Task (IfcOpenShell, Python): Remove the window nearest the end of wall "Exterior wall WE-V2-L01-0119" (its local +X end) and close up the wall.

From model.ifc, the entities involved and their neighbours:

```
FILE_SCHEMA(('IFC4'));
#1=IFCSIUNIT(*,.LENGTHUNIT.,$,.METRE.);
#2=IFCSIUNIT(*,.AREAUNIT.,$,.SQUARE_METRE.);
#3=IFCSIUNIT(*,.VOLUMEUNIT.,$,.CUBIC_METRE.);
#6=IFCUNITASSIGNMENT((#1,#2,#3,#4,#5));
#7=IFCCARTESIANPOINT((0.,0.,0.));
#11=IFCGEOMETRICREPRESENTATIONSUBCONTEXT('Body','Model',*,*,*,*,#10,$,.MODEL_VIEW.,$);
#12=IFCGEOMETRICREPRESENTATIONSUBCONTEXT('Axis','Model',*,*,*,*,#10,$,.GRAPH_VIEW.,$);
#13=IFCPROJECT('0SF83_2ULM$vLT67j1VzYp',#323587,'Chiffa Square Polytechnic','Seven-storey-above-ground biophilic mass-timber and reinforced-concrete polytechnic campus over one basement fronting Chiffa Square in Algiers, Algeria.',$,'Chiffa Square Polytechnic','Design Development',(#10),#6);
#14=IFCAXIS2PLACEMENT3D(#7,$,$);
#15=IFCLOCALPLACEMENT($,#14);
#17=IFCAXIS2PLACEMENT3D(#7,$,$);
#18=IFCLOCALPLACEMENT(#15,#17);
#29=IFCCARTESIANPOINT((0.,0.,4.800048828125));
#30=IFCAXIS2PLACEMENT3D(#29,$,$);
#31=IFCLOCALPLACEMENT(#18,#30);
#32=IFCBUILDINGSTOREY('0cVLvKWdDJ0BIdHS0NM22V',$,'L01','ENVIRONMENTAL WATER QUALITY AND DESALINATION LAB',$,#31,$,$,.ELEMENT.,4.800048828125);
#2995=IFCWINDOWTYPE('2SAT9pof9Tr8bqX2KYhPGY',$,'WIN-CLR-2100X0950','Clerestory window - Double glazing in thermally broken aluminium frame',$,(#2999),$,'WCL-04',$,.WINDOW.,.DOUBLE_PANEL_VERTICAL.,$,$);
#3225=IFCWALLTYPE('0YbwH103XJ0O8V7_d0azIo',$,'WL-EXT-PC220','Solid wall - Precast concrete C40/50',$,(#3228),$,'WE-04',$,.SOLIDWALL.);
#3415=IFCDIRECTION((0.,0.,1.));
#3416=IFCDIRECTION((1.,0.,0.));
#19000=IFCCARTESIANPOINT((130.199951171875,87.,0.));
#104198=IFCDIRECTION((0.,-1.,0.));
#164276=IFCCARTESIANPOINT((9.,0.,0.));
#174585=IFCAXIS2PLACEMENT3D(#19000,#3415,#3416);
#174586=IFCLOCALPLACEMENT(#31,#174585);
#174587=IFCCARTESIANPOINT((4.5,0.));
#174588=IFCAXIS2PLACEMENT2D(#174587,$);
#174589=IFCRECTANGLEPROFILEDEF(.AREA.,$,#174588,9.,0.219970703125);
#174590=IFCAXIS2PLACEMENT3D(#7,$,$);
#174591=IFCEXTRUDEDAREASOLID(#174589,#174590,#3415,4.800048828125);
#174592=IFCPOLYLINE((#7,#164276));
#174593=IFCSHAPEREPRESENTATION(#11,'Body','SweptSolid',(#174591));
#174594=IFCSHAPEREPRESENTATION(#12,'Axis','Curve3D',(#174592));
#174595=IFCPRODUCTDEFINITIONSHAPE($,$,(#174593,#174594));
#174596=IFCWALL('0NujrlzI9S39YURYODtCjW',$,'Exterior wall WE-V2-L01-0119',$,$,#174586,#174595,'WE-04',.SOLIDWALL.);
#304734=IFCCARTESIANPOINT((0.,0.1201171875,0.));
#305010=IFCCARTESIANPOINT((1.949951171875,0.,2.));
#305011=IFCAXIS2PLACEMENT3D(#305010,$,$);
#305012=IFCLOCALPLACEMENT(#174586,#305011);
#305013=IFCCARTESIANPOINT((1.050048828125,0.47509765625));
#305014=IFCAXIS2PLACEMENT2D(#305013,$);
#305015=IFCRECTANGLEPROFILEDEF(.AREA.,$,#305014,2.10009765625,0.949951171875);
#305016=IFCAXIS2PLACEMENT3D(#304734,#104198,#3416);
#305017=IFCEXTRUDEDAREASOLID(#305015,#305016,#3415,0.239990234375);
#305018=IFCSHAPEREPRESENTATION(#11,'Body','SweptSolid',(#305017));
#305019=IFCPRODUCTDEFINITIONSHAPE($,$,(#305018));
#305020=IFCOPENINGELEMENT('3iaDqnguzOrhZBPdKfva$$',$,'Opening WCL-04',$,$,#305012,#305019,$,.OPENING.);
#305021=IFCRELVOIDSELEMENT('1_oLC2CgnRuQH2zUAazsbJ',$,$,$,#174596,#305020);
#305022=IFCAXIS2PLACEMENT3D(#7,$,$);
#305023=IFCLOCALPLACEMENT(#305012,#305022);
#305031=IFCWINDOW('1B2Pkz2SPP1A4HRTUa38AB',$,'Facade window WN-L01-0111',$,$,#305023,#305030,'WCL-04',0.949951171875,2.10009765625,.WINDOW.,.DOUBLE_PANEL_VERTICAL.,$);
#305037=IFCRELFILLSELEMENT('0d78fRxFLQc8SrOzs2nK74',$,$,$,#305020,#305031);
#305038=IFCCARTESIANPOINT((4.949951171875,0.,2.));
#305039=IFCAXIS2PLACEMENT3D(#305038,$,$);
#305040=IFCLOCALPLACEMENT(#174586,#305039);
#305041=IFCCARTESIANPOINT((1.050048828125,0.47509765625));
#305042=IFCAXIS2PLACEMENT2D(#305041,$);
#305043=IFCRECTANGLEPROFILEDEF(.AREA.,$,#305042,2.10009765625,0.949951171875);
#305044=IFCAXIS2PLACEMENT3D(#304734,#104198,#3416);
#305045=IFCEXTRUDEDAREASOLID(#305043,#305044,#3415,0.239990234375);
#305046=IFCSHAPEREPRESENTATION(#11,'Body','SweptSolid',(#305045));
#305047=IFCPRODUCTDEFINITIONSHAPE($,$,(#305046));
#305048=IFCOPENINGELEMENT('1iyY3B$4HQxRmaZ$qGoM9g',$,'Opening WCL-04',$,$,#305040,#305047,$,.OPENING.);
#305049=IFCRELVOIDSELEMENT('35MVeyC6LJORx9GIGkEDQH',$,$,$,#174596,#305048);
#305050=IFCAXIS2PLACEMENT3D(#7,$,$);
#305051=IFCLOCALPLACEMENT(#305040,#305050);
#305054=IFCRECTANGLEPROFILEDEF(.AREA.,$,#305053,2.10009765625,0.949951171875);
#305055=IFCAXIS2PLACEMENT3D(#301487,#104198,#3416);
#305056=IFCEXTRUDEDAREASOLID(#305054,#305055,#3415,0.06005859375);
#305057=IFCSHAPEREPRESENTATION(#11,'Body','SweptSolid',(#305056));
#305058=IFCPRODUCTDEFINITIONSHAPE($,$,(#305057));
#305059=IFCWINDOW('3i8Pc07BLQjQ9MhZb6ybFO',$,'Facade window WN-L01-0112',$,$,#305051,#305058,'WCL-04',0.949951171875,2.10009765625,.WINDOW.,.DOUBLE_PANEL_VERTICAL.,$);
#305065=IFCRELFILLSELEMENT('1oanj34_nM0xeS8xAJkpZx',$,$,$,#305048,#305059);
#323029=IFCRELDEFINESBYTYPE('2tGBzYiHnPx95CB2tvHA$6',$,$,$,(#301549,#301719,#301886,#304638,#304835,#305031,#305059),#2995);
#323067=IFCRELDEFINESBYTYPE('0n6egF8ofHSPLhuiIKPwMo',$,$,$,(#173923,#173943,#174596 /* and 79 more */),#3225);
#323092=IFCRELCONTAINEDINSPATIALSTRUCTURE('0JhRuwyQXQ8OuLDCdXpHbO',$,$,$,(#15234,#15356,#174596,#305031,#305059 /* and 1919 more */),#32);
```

```python
import ifcopenshell
import ifcopenshell.api.feature
import ifcopenshell.api.root
import ifcopenshell.geom
import ifcopenshell.util.shape

model = ifcopenshell.open("model.ifc")
settings = ifcopenshell.geom.settings()


def volume(element):
    """Net volume in cubic metres, openings subtracted."""
    shape = ifcopenshell.geom.create_shape(settings, element)
    return ifcopenshell.util.shape.get_volume(shape.geometry)


window = model.by_guid("3i8Pc07BLQjQ9MhZb6ybFO")
opening = window.FillsVoids[0].RelatingOpeningElement
wall = opening.VoidsElements[0].RelatingBuildingElement
before = volume(wall)

ifcopenshell.api.root.remove_product(model, product=window)
ifcopenshell.api.feature.remove_feature(model, feature=opening)

after = volume(wall)

print(f"wall volume {before:.3f} -> {after:.3f} m3")

model.write("model_edited.ifc")
```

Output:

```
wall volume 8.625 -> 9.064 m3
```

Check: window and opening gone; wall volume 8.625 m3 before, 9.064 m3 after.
